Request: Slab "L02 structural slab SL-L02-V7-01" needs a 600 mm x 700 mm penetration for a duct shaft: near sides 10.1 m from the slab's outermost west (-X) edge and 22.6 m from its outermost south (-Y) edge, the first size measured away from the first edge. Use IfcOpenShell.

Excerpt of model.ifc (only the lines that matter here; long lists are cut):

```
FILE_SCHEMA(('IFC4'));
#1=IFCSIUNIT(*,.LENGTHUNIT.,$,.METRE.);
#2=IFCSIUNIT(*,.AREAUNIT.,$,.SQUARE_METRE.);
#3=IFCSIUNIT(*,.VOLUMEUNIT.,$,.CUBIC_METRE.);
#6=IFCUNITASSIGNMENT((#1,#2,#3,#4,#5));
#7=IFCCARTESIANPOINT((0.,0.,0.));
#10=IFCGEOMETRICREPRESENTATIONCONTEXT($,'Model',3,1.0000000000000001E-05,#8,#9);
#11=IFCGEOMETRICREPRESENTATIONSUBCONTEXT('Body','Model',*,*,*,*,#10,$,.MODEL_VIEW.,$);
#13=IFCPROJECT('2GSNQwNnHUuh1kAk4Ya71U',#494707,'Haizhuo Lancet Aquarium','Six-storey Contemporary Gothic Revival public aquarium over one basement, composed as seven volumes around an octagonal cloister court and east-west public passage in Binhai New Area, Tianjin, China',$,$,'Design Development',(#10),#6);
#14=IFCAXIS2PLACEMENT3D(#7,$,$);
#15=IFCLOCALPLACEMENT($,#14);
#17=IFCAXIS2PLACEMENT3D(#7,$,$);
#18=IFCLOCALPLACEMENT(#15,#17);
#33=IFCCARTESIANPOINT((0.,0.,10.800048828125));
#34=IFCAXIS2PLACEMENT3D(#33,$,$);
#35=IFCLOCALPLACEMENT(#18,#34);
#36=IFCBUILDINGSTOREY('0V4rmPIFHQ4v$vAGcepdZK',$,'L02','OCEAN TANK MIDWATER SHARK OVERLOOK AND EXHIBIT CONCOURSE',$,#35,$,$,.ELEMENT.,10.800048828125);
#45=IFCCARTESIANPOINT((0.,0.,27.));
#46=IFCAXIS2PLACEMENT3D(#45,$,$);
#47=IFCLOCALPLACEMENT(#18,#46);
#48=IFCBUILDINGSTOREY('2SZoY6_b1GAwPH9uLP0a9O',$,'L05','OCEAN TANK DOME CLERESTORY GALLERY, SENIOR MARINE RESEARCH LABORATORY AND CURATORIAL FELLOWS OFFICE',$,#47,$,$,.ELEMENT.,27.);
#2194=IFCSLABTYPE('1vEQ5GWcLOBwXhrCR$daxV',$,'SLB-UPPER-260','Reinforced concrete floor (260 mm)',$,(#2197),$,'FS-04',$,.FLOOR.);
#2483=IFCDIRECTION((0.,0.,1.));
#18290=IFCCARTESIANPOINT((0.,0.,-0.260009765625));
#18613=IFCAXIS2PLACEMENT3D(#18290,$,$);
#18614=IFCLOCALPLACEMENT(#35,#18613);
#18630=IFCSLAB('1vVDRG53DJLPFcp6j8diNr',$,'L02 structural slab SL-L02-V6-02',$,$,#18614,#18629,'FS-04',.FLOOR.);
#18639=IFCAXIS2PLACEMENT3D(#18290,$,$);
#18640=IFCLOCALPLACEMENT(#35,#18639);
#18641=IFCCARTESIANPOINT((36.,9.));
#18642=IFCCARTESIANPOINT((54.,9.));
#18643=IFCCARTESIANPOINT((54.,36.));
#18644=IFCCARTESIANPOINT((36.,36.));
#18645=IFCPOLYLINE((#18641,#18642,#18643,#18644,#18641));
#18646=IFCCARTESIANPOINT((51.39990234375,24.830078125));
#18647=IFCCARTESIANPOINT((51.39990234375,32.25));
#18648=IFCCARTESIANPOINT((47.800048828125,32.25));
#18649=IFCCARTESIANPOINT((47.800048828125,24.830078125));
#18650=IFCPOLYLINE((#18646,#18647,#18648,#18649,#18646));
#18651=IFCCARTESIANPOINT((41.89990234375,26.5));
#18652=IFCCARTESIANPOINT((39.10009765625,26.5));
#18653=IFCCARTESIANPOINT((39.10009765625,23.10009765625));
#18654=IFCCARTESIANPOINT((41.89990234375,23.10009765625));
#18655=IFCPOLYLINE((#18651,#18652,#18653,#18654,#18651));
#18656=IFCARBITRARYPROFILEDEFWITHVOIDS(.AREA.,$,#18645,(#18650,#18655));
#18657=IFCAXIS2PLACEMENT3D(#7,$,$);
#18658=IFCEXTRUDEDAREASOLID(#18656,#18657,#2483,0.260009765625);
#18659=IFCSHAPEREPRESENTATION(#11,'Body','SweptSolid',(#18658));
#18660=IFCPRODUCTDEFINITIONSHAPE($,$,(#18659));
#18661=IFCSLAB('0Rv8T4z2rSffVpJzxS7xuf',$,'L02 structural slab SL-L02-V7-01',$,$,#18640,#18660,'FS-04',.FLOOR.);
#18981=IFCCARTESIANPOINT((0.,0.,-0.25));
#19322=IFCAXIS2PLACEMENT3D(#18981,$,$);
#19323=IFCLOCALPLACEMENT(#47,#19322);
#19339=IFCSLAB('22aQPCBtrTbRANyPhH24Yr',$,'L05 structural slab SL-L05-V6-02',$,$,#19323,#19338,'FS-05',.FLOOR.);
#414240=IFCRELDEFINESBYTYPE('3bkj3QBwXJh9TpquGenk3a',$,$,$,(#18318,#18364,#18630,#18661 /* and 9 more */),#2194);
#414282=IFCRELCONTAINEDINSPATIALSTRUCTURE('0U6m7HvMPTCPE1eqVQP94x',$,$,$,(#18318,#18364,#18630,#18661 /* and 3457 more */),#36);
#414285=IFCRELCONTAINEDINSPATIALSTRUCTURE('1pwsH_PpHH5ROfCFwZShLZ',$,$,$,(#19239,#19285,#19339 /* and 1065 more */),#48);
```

```python
import numpy as np
import ifcopenshell
import ifcopenshell.api.feature
import ifcopenshell.api.geometry
import ifcopenshell.api.root
import ifcopenshell.geom
import ifcopenshell.util.placement
import ifcopenshell.util.representation
import ifcopenshell.util.shape
import ifcopenshell.util.unit

model = ifcopenshell.open("model.ifc")
unit_scale = ifcopenshell.util.unit.calculate_unit_scale(model)
settings = ifcopenshell.geom.settings()


def volume(element):
    """Net volume in cubic metres, openings subtracted."""
    shape = ifcopenshell.geom.create_shape(settings, element)
    return ifcopenshell.util.shape.get_volume(shape.geometry)


slab = model.by_guid("0Rv8T4z2rSffVpJzxS7xuf")
before = volume(slab)

# Extent in the slab's own axes, in metres. The edges named are its -X and -Y sides.
slab_shape = ifcopenshell.geom.create_shape(settings, slab)
vertices = ifcopenshell.util.shape.get_vertices(slab_shape.geometry)
x_min, y_min, bottom = vertices.min(axis=0)
top = vertices[:, 2].max()

opening = ifcopenshell.api.root.create_entity(model, ifc_class="IfcOpeningElement", name="Duct shaft opening", predefined_type="OPENING")
context = ifcopenshell.util.representation.get_context(model, "Model", "Body", "MODEL_VIEW")
width, depth = 0.6, 0.7
outline = [(0.0, 0.0), (width, 0.0), (width, depth), (0.0, depth), (0.0, 0.0)]
# Overshoot both faces by 50 mm so the cut is clean.
shape = ifcopenshell.api.geometry.add_slab_representation(
    model, context=context, depth=top - bottom + 0.1, polyline=outline
)
ifcopenshell.api.geometry.assign_representation(model, product=opening, representation=shape)

matrix = ifcopenshell.util.placement.get_local_placement(slab.ObjectPlacement)
matrix[:, 3] = matrix @ np.append(np.array([x_min + 10.1, y_min + 22.6, bottom - 0.05]) / unit_scale, 1.0)
ifcopenshell.api.geometry.edit_object_placement(model, product=opening, matrix=matrix, is_si=False)
ifcopenshell.api.feature.add_feature(model, feature=opening, element=slab)

after = volume(slab)

print(f"slab volume {before:.3f} -> {after:.3f} m3")

model.write("model_rev.ifc")
```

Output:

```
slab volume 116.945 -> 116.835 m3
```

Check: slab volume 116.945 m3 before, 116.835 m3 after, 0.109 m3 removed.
